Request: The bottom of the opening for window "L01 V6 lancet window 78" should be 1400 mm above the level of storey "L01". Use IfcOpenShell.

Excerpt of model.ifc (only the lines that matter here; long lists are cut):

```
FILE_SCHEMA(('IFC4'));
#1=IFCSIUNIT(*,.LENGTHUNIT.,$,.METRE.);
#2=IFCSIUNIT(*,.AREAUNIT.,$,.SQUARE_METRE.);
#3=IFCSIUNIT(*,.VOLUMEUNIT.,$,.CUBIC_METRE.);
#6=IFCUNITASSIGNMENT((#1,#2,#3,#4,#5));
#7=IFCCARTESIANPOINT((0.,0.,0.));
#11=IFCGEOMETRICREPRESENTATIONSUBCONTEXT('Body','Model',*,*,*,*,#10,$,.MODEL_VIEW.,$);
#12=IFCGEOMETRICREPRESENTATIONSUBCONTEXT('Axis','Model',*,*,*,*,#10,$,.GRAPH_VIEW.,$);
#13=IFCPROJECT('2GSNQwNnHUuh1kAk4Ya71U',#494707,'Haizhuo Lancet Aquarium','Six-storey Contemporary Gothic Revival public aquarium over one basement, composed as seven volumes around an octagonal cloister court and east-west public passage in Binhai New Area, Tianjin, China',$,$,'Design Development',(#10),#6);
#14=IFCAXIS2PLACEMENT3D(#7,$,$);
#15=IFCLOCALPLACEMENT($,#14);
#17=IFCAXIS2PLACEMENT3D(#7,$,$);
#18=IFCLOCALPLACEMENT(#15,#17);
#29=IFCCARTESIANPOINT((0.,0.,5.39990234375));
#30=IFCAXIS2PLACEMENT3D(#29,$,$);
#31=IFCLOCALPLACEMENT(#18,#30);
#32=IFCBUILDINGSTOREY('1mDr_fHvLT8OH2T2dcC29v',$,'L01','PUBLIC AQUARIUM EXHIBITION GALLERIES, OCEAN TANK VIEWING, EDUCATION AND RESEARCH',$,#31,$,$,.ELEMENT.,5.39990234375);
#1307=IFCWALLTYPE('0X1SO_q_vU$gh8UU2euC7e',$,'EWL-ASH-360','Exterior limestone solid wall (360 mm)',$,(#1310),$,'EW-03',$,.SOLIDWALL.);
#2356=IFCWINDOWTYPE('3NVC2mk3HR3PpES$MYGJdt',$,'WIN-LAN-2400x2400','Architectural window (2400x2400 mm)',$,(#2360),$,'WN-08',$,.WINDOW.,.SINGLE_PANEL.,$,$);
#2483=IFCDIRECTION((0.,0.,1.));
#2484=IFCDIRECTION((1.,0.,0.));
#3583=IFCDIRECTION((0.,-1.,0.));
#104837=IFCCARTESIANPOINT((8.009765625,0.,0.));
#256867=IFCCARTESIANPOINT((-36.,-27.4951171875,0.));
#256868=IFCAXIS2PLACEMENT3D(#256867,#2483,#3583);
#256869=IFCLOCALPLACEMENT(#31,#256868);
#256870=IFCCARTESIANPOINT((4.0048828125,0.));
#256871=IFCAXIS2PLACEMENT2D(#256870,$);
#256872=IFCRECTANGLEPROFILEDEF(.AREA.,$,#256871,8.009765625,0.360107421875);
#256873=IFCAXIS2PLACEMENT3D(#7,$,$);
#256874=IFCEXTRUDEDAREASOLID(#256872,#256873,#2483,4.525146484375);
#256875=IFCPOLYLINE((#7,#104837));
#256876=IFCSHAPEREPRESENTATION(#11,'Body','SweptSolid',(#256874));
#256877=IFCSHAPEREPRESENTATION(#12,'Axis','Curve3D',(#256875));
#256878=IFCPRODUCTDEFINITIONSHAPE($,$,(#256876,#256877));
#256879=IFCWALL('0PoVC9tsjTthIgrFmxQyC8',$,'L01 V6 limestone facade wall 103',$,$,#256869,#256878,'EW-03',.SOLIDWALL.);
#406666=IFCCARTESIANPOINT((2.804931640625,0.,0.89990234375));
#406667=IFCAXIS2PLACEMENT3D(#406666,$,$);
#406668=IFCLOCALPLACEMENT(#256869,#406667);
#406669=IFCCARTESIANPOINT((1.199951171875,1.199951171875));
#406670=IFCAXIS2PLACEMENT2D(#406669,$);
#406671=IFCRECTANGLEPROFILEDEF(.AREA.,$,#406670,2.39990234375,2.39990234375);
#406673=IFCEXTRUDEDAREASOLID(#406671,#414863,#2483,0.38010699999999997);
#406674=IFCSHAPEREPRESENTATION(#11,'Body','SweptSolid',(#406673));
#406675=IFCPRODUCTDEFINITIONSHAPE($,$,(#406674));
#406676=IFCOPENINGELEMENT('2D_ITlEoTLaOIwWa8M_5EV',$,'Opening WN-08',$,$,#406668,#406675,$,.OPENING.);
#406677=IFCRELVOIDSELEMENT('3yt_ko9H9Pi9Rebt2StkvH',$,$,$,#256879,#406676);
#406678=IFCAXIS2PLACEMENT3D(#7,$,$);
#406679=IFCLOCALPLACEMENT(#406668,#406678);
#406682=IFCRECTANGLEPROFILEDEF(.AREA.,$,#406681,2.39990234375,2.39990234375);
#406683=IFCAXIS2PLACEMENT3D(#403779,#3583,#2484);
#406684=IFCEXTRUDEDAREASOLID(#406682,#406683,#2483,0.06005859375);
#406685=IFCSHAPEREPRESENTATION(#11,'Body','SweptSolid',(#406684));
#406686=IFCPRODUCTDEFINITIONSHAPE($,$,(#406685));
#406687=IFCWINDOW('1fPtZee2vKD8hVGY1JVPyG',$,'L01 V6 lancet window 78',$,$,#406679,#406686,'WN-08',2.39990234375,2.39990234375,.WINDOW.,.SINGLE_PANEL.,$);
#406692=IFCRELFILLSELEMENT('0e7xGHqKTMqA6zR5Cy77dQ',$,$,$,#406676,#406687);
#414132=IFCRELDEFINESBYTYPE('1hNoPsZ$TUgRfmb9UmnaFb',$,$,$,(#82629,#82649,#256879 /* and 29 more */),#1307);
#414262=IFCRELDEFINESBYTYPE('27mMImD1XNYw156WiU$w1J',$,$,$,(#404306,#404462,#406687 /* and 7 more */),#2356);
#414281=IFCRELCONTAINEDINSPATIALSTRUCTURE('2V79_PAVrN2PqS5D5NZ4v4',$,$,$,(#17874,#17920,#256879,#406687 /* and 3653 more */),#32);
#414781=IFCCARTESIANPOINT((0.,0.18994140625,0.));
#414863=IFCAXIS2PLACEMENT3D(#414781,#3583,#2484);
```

```python
import numpy as np
import ifcopenshell
import ifcopenshell.api.geometry
import ifcopenshell.geom
import ifcopenshell.util.element
import ifcopenshell.util.placement
import ifcopenshell.util.shape
import ifcopenshell.util.unit

model = ifcopenshell.open("model.ifc")
unit_scale = ifcopenshell.util.unit.calculate_unit_scale(model)

window = model.by_id(406687)
opening = window.FillsVoids[0].RelatingOpeningElement
storey = ifcopenshell.util.element.get_container(window, ifc_class="IfcBuildingStorey")
level = ifcopenshell.util.placement.get_local_placement(storey.ObjectPlacement)[2, 3]

# The opening's origin need not be at the sill, so measure its lowest point.
shape = ifcopenshell.geom.create_shape(ifcopenshell.geom.settings(), opening)
bottom = ifcopenshell.util.shape.get_shape_bottom_elevation(shape, shape.geometry) / unit_scale
dz = level + 1.4 / unit_scale - bottom

shift = np.array([0.0, 0.0, dz])
# The window is placed relative to its opening, so it follows when the opening moves.
matrix = ifcopenshell.util.placement.get_local_placement(opening.ObjectPlacement)
matrix[:3, 3] += shift
ifcopenshell.api.geometry.edit_object_placement(
    model, product=opening, matrix=matrix, is_si=False, should_transform_children=True
)

print(f"moved by {dz * unit_scale:+.3f} m")

model.write("model_updated.ifc")
```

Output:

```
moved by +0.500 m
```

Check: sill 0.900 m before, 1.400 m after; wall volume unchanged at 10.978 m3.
